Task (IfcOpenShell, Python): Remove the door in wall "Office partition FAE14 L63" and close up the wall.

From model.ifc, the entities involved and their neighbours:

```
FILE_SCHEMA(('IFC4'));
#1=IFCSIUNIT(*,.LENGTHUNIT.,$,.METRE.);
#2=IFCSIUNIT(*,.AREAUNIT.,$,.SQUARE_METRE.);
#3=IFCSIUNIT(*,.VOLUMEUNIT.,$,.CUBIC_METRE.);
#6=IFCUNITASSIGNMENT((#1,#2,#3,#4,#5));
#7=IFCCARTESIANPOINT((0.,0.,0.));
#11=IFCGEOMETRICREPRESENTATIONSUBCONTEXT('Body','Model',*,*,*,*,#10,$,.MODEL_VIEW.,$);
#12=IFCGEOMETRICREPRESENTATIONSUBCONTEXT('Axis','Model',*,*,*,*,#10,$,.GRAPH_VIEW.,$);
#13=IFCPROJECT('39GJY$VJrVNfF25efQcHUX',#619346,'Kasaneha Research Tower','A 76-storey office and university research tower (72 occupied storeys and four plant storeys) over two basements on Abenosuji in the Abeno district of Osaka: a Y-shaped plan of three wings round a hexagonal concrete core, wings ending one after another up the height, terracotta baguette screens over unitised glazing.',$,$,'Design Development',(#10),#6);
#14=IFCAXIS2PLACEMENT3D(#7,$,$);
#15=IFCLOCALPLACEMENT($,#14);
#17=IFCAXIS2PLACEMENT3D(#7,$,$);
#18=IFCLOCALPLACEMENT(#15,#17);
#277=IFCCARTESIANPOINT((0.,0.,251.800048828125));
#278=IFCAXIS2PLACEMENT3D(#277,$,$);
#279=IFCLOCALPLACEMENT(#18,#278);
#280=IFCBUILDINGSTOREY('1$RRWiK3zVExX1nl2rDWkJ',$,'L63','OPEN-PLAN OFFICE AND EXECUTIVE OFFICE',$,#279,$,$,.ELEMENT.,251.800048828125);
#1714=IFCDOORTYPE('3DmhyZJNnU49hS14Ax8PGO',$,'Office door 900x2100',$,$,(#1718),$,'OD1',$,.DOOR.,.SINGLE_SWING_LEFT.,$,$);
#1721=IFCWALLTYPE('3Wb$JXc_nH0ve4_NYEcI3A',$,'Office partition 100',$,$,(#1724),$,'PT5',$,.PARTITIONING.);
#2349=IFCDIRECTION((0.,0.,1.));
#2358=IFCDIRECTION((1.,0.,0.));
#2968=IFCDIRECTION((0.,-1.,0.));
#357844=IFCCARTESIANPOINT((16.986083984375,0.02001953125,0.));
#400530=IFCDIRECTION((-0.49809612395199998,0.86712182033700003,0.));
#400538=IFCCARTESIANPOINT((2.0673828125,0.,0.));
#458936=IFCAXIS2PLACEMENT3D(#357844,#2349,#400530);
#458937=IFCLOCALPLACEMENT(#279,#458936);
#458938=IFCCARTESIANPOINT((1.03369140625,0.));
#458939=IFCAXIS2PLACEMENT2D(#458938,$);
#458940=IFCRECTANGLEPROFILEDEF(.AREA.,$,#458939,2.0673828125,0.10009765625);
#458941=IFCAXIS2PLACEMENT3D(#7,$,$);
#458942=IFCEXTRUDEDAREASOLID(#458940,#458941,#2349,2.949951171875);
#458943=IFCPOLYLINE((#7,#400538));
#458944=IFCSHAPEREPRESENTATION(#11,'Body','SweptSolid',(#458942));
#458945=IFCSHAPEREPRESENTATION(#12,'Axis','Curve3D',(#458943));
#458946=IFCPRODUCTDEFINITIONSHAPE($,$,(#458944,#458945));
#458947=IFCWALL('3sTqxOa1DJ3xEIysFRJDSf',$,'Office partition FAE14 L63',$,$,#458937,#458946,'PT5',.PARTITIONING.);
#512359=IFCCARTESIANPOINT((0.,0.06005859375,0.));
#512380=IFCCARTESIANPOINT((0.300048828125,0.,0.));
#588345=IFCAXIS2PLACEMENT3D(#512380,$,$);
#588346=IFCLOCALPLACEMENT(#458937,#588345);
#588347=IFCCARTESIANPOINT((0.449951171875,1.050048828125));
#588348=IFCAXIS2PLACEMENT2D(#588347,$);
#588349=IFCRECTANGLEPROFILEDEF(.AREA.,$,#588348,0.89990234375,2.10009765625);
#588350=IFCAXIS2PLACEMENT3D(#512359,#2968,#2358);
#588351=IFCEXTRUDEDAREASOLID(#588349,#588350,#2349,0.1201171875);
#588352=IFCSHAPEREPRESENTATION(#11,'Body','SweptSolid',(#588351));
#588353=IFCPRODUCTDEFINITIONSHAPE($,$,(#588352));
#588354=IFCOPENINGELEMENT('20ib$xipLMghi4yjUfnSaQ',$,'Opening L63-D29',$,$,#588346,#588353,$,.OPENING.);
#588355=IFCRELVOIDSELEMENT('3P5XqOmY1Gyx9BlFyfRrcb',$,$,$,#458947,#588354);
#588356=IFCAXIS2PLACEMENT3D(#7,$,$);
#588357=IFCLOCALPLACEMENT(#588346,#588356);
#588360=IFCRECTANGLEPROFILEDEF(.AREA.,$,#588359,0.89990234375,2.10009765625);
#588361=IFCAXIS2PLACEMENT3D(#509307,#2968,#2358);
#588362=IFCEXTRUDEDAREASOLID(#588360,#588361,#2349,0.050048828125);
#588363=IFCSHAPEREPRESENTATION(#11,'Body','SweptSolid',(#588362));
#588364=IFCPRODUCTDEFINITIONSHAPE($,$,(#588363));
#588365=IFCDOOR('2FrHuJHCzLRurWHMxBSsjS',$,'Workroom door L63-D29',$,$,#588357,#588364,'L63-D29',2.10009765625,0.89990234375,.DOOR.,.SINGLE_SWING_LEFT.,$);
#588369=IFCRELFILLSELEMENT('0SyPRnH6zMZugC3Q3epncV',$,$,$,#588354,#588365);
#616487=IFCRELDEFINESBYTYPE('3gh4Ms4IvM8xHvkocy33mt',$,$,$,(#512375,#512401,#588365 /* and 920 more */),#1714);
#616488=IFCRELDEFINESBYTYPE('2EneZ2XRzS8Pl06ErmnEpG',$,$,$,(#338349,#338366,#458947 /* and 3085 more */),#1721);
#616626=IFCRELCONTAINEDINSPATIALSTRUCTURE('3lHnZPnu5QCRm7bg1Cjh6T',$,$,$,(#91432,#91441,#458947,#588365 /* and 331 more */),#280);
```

```python
import ifcopenshell
import ifcopenshell.api.feature
import ifcopenshell.api.root
import ifcopenshell.geom
import ifcopenshell.util.shape

model = ifcopenshell.open("model.ifc")
settings = ifcopenshell.geom.settings()


def volume(element):
    """Net volume in cubic metres, openings subtracted."""
    shape = ifcopenshell.geom.create_shape(settings, element)
    return ifcopenshell.util.shape.get_volume(shape.geometry)


door = model.by_guid("2FrHuJHCzLRurWHMxBSsjS")
opening = door.FillsVoids[0].RelatingOpeningElement
wall = opening.VoidsElements[0].RelatingBuildingElement
before = volume(wall)

ifcopenshell.api.root.remove_product(model, product=door)
ifcopenshell.api.feature.remove_feature(model, feature=opening)

after = volume(wall)

print(f"wall volume {before:.3f} -> {after:.3f} m3")

model.write("model_edited.ifc")
```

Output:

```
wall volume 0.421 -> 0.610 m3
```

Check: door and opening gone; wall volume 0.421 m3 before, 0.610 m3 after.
